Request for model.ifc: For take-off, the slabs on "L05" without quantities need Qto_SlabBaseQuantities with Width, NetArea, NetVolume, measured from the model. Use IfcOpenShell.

First a look at what the model holds.

```python
import ifcopenshell
import ifcopenshell.util.element
import ifcopenshell.util.unit

model = ifcopenshell.open("model.ifc")
print(model.schema)
for unit_type in ("LENGTHUNIT", "AREAUNIT", "VOLUMEUNIT"):
    print(unit_type, ifcopenshell.util.unit.calculate_unit_scale(model, unit_type))
storey = next(s for s in model.by_type("IfcBuildingStorey") if s.Name == "L05")
slabs = [e for e in ifcopenshell.util.element.get_decomposition(storey) if e.is_a("IfcSlab")]
for e in sorted(slabs, key=lambda e: e.id()):
    print(e.id(), e.is_a(), e.Name, list(ifcopenshell.util.element.get_psets(e, qtos_only=True)), sep=" | ")
```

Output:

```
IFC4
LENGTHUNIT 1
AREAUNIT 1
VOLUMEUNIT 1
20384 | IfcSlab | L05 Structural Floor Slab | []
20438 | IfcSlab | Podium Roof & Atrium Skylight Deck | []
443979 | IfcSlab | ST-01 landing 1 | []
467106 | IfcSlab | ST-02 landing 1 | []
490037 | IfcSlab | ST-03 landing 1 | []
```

```python
import ifcopenshell
import ifcopenshell.api.pset
import ifcopenshell.geom
import ifcopenshell.util.element
import ifcopenshell.util.shape
import ifcopenshell.util.unit

model = ifcopenshell.open("model.ifc")
unit_scale = ifcopenshell.util.unit.calculate_unit_scale(model)
area_scale = ifcopenshell.util.unit.calculate_unit_scale(model, "AREAUNIT")
volume_scale = ifcopenshell.util.unit.calculate_unit_scale(model, "VOLUMEUNIT")
settings = ifcopenshell.geom.settings()

storey = next(s for s in model.by_type("IfcBuildingStorey") if s.Name == "L05")
slabs = [e for e in ifcopenshell.util.element.get_decomposition(storey) if e.is_a("IfcSlab")]

for e in sorted(slabs, key=lambda e: e.id()):
    if ifcopenshell.util.element.get_psets(e, qtos_only=True, should_inherit=False):
        continue
    # Geometry comes back in metres, in the element's own axes.
    shape = ifcopenshell.geom.create_shape(settings, e)
    values = {
        "Width": ifcopenshell.util.shape.get_z(shape.geometry) / unit_scale,
        "NetArea": ifcopenshell.util.shape.get_footprint_area(shape.geometry) / area_scale,
        "NetVolume": ifcopenshell.util.shape.get_volume(shape.geometry) / volume_scale,
    }
    qto = ifcopenshell.api.pset.add_qto(model, product=e, name="Qto_SlabBaseQuantities")
    ifcopenshell.api.pset.edit_qto(model, qto=qto, properties=values)
    print(e.id(), {k: round(v, 3) for k, v in values.items()})

model.write("model_updated.ifc")
```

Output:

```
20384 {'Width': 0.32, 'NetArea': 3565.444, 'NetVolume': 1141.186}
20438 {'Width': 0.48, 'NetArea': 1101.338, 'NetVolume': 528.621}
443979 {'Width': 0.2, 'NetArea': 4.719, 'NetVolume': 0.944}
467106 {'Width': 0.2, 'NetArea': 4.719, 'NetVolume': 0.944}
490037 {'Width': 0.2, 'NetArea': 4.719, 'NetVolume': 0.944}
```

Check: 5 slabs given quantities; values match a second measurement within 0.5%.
